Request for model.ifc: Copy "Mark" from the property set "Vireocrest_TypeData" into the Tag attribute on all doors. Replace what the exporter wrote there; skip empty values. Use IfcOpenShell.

First a look at what the model holds.

```python
import ifcopenshell
import ifcopenshell.util.element

model = ifcopenshell.open("model.ifc")
print(model.schema)
doors = model.by_type("IfcDoor")
print(len(doors), "doors")
for e in doors[:8]:
    source = ifcopenshell.util.element.get_pset(e, "Vireocrest_TypeData", "Mark")
    target = e.Tag
    print(e.id(), repr(source), repr(target), sep=" | ")
```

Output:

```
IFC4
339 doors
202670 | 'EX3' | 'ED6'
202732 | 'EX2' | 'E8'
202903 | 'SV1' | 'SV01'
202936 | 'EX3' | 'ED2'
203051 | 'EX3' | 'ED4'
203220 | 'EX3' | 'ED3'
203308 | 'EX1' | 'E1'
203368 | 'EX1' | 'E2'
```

```python
import ifcopenshell
import ifcopenshell.util.element

model = ifcopenshell.open("model.ifc")

count = 0
for e in model.by_type("IfcDoor"):
    value = ifcopenshell.util.element.get_pset(e, "Vireocrest_TypeData", "Mark")
    current = e.Tag
    if not value or not value.strip() or current == value:
        continue
    e.Tag = value
    count += 1

print(count, "doors updated")

model.write("model_updated.ifc")
```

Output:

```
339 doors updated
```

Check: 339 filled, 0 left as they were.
